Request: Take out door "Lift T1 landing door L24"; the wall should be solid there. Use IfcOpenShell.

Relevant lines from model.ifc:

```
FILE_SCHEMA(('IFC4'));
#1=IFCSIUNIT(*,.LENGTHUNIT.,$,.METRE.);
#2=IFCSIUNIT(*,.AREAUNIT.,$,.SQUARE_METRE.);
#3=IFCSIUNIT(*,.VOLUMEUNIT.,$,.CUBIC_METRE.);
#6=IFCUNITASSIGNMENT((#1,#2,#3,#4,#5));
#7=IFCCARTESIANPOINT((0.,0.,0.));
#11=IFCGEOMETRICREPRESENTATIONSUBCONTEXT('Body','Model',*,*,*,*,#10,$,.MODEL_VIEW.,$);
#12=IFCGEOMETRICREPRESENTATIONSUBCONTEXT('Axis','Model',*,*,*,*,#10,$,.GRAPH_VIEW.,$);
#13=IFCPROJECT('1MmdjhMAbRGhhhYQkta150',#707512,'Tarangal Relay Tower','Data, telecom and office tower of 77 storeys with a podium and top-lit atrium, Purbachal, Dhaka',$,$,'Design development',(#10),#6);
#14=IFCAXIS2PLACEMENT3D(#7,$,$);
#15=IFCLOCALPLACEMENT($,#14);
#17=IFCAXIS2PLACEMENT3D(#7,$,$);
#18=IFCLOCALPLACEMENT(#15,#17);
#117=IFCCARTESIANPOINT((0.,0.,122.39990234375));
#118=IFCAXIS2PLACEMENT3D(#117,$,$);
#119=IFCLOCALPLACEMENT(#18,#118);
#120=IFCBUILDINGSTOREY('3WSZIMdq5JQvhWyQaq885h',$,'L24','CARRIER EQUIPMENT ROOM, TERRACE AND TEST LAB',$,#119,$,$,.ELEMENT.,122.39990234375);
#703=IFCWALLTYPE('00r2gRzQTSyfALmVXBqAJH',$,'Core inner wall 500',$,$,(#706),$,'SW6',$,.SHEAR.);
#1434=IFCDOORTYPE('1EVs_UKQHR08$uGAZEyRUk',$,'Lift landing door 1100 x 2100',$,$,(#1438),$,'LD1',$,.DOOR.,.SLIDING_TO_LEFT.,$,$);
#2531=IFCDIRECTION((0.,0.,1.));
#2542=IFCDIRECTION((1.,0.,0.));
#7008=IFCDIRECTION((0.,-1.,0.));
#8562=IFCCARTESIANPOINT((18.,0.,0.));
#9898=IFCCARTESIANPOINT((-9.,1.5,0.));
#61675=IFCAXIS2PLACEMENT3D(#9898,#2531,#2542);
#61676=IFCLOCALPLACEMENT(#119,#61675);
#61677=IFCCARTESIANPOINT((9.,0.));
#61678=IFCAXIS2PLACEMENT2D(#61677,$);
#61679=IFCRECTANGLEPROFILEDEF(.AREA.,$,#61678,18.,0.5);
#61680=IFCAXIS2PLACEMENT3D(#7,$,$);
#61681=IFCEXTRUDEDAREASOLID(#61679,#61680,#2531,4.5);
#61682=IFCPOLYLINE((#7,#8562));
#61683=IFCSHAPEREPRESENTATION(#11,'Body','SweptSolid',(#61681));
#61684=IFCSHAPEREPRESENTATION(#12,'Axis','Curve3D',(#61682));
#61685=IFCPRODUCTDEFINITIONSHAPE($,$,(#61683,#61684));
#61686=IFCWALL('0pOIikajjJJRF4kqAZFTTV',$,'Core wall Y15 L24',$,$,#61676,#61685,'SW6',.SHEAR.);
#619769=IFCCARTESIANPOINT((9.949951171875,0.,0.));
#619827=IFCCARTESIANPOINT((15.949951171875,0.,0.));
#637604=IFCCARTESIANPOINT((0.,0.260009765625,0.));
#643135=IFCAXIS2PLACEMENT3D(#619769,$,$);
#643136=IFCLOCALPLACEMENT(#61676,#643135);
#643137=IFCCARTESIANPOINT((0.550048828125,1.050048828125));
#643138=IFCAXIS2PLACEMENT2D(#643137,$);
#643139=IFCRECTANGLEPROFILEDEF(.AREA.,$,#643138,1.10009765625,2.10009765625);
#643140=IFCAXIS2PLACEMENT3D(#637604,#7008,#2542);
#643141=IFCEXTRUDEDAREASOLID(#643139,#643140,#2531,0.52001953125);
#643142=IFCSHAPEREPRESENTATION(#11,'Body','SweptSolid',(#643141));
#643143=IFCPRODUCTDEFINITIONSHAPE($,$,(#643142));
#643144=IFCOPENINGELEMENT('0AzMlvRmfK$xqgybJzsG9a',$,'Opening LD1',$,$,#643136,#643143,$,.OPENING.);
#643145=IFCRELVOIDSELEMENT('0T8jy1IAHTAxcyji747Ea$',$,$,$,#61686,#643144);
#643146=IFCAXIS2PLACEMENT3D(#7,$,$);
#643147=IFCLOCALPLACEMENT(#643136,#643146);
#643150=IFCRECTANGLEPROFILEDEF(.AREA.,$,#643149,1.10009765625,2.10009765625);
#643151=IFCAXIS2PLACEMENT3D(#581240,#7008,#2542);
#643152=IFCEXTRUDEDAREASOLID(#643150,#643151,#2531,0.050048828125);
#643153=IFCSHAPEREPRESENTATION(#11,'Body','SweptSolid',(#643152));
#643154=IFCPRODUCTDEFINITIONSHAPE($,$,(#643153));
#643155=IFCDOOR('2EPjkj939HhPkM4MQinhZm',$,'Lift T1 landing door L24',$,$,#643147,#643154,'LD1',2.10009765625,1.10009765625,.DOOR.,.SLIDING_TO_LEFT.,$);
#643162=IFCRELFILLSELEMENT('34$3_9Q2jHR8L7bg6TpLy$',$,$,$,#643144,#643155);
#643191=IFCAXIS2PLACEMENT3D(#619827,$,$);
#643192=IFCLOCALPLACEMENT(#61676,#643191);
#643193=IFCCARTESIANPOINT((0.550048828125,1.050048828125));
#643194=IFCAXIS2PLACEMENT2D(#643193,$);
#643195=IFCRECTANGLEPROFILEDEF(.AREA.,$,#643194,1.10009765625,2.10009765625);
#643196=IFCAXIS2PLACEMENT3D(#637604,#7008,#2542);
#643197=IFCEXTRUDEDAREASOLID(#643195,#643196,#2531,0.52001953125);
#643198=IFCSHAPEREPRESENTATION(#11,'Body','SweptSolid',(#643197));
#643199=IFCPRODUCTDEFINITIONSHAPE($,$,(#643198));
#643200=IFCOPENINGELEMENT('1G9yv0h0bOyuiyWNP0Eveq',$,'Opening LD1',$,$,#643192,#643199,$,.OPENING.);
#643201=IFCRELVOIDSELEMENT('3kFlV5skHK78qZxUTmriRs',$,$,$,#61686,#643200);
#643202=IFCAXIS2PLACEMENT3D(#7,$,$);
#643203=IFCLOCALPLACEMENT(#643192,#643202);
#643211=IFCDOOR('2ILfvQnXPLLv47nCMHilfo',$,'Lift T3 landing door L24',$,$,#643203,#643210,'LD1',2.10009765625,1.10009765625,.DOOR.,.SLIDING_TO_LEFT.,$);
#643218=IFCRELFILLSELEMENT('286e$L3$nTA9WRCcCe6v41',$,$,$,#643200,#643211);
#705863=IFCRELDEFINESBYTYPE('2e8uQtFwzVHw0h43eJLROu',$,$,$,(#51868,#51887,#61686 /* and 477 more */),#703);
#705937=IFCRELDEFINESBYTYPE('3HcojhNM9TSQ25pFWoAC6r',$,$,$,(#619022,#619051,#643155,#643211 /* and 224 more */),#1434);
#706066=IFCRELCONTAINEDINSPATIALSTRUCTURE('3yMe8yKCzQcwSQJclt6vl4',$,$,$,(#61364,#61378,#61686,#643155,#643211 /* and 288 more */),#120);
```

```python
import ifcopenshell
import ifcopenshell.api.feature
import ifcopenshell.api.root
import ifcopenshell.geom
import ifcopenshell.util.shape

model = ifcopenshell.open("model.ifc")
settings = ifcopenshell.geom.settings()


def volume(element):
    """Net volume in cubic metres, openings subtracted."""
    shape = ifcopenshell.geom.create_shape(settings, element)
    return ifcopenshell.util.shape.get_volume(shape.geometry)


door = model.by_id(643155)
opening = door.FillsVoids[0].RelatingOpeningElement
wall = opening.VoidsElements[0].RelatingBuildingElement
before = volume(wall)

ifcopenshell.api.root.remove_product(model, product=door)
ifcopenshell.api.feature.remove_feature(model, feature=opening)

after = volume(wall)

print(f"wall volume {before:.3f} -> {after:.3f} m3")

model.write("model_v2.ifc")
```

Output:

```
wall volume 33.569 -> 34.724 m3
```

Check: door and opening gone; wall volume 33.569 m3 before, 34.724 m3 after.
